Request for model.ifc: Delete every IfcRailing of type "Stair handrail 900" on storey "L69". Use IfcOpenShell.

First a look at what the model holds.

```python
import ifcopenshell
import ifcopenshell.util.element

model = ifcopenshell.open("model.ifc")
print(model.schema)
storey = next(s for s in model.by_type("IfcBuildingStorey") if s.Name == "L69")
railings = [e for e in ifcopenshell.util.element.get_decomposition(storey) if e.is_a("IfcRailing")]
seen = {}
for e in railings:
    element_type = ifcopenshell.util.element.get_type(e)
    name = element_type.Name if element_type not in (None, e) else None
    seen[name] = seen.get(name, 0) + 1
for name, count in sorted(seen.items(), key=str):
    print(count, "x", name)
```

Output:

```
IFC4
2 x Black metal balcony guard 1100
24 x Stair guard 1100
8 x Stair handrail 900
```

```python
import ifcopenshell
import ifcopenshell.api.root
import ifcopenshell.util.element

model = ifcopenshell.open("model.ifc")

storey = next(s for s in model.by_type("IfcBuildingStorey") if s.Name == "L69")
railings = [e for e in ifcopenshell.util.element.get_decomposition(storey) if e.is_a("IfcRailing")]
targets = [e for e in railings if (t := ifcopenshell.util.element.get_type(e)) not in (None, e) and t.Name == "Stair handrail 900"]

for e in targets:
    ifcopenshell.api.root.remove_product(model, product=e)
print(len(targets), "removed")

model.write("model_v2.ifc")
```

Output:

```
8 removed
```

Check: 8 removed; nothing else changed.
